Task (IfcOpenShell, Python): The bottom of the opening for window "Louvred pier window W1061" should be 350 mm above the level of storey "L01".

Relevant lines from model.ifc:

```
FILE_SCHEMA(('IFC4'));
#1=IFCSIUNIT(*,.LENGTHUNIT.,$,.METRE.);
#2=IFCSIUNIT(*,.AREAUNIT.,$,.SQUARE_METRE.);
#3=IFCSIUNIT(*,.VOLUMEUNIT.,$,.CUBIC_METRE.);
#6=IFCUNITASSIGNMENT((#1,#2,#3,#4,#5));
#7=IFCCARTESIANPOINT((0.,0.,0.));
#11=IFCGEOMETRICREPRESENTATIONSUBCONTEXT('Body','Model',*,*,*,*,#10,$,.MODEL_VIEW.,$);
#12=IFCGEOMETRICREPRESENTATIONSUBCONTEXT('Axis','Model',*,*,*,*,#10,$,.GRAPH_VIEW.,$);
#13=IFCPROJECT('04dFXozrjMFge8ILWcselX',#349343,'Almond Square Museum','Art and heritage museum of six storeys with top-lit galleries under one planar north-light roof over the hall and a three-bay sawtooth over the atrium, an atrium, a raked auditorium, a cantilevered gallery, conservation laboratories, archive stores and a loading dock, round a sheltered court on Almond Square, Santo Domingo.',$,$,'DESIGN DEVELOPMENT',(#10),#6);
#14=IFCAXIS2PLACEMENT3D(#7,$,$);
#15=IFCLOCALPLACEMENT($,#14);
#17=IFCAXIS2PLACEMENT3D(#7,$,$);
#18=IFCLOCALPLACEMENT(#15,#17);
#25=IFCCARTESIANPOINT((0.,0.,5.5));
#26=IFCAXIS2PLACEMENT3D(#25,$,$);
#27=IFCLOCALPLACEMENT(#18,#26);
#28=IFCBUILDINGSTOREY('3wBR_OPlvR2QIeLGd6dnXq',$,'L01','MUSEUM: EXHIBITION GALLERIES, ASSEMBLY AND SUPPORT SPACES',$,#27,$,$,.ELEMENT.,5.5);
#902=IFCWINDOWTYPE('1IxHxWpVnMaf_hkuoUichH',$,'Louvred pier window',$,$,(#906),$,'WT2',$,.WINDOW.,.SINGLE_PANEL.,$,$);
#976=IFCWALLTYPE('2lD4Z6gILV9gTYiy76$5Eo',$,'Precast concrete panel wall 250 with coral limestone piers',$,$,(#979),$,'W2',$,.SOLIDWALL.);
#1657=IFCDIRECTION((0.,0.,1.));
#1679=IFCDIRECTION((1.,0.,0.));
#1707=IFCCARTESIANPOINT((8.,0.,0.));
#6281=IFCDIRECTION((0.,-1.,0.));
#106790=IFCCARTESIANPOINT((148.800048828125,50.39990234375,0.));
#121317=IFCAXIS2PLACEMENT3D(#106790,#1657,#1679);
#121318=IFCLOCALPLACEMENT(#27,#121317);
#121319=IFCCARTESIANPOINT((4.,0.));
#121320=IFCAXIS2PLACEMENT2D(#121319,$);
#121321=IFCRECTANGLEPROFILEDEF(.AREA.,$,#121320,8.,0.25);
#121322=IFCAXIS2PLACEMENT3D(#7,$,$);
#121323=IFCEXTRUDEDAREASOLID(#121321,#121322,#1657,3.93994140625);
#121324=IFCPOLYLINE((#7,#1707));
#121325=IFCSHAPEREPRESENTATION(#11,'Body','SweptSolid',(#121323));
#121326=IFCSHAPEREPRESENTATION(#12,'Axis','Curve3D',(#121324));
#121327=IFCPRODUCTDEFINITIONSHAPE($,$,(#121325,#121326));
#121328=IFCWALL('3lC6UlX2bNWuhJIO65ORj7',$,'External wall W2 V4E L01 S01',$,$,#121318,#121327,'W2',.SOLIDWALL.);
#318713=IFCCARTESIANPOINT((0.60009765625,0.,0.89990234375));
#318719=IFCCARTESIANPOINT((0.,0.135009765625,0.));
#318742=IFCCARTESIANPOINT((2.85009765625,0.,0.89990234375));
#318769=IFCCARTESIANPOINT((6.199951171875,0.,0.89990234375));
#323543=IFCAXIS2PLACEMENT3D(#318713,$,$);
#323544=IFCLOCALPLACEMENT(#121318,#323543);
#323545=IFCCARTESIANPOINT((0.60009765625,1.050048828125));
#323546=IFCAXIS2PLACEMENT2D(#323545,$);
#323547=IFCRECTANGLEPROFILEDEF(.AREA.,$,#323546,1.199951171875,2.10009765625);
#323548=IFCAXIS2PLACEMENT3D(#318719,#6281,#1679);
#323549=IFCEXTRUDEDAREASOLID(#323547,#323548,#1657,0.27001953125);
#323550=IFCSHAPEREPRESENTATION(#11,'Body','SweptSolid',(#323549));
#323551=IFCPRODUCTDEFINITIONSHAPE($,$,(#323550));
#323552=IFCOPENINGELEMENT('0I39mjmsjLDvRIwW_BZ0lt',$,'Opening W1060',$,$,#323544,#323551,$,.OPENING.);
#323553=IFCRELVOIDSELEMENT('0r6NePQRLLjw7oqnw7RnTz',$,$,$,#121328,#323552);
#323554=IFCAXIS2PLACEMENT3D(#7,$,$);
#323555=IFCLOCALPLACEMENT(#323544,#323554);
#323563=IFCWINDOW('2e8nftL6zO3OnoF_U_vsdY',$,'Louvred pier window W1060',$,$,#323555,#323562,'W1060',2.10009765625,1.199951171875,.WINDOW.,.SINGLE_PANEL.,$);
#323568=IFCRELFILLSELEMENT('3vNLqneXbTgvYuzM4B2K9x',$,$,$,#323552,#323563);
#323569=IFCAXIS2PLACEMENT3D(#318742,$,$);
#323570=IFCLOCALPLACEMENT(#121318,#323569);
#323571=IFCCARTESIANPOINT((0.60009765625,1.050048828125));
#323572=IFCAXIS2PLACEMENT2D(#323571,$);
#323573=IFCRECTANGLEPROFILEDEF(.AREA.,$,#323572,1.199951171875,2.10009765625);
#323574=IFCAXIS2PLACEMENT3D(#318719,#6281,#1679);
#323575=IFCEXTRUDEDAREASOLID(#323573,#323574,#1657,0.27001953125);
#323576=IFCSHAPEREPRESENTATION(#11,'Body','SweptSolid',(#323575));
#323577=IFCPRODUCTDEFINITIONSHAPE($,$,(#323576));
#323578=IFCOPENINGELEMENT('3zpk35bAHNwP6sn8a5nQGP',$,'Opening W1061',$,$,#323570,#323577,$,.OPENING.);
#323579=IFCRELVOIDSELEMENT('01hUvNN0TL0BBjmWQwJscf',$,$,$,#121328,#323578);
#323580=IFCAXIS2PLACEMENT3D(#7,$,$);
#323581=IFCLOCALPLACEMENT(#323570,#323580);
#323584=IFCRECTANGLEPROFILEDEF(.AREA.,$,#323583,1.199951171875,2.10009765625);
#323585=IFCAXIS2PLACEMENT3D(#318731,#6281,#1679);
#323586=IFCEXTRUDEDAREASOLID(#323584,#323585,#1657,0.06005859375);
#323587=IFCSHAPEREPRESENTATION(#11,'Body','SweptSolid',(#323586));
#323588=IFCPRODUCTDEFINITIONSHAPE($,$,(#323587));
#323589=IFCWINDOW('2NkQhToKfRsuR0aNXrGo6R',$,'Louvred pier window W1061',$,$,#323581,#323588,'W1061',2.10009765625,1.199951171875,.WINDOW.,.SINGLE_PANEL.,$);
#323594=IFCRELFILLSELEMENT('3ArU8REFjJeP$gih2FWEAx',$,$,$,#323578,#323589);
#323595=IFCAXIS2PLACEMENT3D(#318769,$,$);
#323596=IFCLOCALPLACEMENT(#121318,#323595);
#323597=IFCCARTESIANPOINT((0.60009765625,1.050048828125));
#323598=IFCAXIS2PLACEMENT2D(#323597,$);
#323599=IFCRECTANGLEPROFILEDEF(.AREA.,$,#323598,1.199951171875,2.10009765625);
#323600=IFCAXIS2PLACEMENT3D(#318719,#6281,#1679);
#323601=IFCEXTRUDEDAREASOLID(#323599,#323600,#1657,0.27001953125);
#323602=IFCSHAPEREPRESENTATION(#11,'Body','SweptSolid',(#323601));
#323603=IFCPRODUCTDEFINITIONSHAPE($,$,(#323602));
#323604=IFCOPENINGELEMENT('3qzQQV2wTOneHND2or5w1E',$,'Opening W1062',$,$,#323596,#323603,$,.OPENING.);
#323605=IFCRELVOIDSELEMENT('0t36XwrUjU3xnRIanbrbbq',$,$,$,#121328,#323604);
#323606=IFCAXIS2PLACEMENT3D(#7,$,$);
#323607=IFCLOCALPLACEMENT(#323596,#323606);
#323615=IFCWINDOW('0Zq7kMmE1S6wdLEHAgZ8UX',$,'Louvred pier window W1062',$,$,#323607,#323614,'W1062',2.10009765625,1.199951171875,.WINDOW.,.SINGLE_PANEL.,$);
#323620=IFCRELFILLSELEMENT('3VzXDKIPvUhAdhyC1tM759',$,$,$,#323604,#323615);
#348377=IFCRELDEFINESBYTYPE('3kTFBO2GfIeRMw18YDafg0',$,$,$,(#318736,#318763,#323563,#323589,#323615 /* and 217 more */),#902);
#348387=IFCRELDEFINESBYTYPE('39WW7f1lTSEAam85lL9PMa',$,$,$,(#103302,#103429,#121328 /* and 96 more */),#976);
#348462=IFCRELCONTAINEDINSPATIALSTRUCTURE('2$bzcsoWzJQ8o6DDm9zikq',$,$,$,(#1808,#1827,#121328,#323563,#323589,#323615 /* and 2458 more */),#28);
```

```python
import numpy as np
import ifcopenshell
import ifcopenshell.api.geometry
import ifcopenshell.geom
import ifcopenshell.util.element
import ifcopenshell.util.placement
import ifcopenshell.util.shape
import ifcopenshell.util.unit

model = ifcopenshell.open("model.ifc")
unit_scale = ifcopenshell.util.unit.calculate_unit_scale(model)

window = model.by_guid("2NkQhToKfRsuR0aNXrGo6R")
opening = window.FillsVoids[0].RelatingOpeningElement
storey = ifcopenshell.util.element.get_container(window, ifc_class="IfcBuildingStorey")
level = ifcopenshell.util.placement.get_local_placement(storey.ObjectPlacement)[2, 3]

# The opening's origin need not be at the sill, so measure its lowest point.
shape = ifcopenshell.geom.create_shape(ifcopenshell.geom.settings(), opening)
bottom = ifcopenshell.util.shape.get_shape_bottom_elevation(shape, shape.geometry) / unit_scale
dz = level + 0.35 - bottom

shift = np.array([0.0, 0.0, dz])
# The window is placed relative to its opening, so it follows when the opening moves.
matrix = ifcopenshell.util.placement.get_local_placement(opening.ObjectPlacement)
matrix[:3, 3] += shift
ifcopenshell.api.geometry.edit_object_placement(
    model, product=opening, matrix=matrix, is_si=False, should_transform_children=True
)

print(f"moved by {dz * unit_scale:+.3f} m")

model.write("model_edited.ifc")
```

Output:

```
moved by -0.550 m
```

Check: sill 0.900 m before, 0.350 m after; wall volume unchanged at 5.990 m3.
